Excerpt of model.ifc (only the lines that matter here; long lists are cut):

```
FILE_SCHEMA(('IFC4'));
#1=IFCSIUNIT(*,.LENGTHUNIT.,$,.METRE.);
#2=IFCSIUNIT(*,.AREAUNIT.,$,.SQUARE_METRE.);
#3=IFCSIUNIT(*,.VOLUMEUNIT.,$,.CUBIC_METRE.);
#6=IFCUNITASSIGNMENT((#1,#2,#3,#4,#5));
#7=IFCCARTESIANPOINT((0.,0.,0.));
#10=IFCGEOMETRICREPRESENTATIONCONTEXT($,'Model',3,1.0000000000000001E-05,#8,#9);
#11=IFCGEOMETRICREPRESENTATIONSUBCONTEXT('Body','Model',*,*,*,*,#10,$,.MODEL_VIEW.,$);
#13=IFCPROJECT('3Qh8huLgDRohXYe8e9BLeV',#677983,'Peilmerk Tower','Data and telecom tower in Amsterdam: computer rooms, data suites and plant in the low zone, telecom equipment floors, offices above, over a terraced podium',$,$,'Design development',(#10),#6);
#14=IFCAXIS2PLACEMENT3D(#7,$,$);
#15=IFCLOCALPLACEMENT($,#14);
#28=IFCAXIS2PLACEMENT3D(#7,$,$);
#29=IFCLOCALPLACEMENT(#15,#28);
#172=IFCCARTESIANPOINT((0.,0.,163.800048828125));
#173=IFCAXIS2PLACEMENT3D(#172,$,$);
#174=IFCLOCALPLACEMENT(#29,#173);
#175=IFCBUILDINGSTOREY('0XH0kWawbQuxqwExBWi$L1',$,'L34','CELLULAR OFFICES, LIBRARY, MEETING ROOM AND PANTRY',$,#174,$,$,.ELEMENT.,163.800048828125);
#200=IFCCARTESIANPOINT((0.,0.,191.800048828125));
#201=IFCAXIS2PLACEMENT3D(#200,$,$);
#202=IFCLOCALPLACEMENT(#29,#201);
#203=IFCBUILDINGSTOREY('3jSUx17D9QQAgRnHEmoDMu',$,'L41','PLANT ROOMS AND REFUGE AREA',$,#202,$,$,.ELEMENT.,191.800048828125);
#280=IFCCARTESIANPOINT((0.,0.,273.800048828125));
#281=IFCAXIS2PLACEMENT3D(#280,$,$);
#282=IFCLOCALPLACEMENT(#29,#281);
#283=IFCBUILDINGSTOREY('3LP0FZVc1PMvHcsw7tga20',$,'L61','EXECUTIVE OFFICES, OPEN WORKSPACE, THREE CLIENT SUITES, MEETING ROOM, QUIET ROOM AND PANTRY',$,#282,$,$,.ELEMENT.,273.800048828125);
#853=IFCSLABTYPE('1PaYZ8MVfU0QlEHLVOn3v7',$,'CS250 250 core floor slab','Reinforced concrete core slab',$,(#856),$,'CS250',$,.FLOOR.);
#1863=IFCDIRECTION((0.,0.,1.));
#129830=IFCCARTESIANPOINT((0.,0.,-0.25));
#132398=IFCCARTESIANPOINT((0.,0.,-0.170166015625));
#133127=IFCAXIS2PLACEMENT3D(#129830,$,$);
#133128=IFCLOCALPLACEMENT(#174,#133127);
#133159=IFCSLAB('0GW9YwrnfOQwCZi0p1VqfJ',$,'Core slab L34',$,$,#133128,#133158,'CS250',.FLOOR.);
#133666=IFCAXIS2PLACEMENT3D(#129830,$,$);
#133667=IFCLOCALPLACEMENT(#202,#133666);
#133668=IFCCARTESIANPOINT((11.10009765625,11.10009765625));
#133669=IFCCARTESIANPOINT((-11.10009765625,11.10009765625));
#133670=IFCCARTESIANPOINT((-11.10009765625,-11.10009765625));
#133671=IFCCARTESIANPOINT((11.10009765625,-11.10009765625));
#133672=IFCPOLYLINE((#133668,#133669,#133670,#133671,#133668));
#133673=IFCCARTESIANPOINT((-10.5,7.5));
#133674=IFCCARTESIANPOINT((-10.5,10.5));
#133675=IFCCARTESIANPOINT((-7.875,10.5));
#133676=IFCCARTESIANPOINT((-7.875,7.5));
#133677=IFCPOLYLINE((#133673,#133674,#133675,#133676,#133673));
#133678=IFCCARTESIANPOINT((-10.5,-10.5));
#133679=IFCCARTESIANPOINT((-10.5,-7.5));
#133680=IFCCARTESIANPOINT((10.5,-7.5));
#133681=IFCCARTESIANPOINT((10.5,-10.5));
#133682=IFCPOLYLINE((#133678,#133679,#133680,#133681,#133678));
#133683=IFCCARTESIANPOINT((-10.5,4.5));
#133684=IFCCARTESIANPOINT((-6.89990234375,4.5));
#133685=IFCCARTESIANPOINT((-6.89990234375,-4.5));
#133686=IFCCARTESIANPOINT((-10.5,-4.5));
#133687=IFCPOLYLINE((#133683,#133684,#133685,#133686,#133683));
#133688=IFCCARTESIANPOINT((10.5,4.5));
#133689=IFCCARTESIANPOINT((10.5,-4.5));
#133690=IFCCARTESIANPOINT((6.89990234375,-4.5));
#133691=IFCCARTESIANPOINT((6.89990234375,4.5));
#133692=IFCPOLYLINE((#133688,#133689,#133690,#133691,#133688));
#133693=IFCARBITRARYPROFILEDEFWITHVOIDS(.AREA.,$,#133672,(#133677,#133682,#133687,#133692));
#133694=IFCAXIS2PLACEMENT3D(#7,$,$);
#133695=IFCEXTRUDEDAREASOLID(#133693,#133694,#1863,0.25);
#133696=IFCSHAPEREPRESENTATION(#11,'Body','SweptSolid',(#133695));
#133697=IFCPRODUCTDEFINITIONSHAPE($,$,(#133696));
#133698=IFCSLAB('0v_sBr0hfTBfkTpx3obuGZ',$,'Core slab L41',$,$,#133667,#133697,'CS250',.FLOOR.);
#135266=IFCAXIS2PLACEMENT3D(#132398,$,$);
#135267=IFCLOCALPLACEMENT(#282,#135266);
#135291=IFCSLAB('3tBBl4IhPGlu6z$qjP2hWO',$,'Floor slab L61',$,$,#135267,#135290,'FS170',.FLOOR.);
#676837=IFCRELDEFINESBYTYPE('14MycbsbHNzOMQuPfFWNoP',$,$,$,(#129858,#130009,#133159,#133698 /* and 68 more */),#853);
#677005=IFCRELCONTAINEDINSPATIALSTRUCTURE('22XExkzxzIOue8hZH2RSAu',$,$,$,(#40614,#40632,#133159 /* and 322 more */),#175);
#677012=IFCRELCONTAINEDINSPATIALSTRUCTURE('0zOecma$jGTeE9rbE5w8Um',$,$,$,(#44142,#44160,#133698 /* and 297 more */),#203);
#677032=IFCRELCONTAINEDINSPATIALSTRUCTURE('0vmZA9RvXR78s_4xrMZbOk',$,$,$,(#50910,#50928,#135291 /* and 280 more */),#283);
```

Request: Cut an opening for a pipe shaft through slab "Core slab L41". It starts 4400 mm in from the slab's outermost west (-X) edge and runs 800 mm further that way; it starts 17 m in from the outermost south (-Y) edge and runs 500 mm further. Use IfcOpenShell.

```python
import numpy as np
import ifcopenshell
import ifcopenshell.api.feature
import ifcopenshell.api.geometry
import ifcopenshell.api.root
import ifcopenshell.geom
import ifcopenshell.util.placement
import ifcopenshell.util.representation
import ifcopenshell.util.shape
import ifcopenshell.util.unit

model = ifcopenshell.open("model.ifc")
unit_scale = ifcopenshell.util.unit.calculate_unit_scale(model)
settings = ifcopenshell.geom.settings()


def volume(element):
    """Net volume in cubic metres, openings subtracted."""
    shape = ifcopenshell.geom.create_shape(settings, element)
    return ifcopenshell.util.shape.get_volume(shape.geometry)


slab = model.by_guid("0v_sBr0hfTBfkTpx3obuGZ")
before = volume(slab)

# Extent in the slab's own axes, in metres. The edges named are its -X and -Y sides.
slab_shape = ifcopenshell.geom.create_shape(settings, slab)
vertices = ifcopenshell.util.shape.get_vertices(slab_shape.geometry)
x_min, y_min, bottom = vertices.min(axis=0)
top = vertices[:, 2].max()

opening = ifcopenshell.api.root.create_entity(model, ifc_class="IfcOpeningElement", name="Pipe shaft opening", predefined_type="OPENING")
context = ifcopenshell.util.representation.get_context(model, "Model", "Body", "MODEL_VIEW")
width, depth = 0.8, 0.5
outline = [(0.0, 0.0), (width, 0.0), (width, depth), (0.0, depth), (0.0, 0.0)]
# Overshoot both faces by 50 mm so the cut is clean.
shape = ifcopenshell.api.geometry.add_slab_representation(
    model, context=context, depth=top - bottom + 0.1, polyline=outline
)
ifcopenshell.api.geometry.assign_representation(model, product=opening, representation=shape)

matrix = ifcopenshell.util.placement.get_local_placement(slab.ObjectPlacement)
matrix[:, 3] = matrix @ np.append(np.array([x_min + 4.4, y_min + 17, bottom - 0.05]) / unit_scale, 1.0)
ifcopenshell.api.geometry.edit_object_placement(model, product=opening, matrix=matrix, is_si=False)
ifcopenshell.api.feature.add_feature(model, feature=opening, element=slab)

after = volume(slab)

print(f"slab volume {before:.3f} -> {after:.3f} m3")

model.write("model_edited.ifc")
```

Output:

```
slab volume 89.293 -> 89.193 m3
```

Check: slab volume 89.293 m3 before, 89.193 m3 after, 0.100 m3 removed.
